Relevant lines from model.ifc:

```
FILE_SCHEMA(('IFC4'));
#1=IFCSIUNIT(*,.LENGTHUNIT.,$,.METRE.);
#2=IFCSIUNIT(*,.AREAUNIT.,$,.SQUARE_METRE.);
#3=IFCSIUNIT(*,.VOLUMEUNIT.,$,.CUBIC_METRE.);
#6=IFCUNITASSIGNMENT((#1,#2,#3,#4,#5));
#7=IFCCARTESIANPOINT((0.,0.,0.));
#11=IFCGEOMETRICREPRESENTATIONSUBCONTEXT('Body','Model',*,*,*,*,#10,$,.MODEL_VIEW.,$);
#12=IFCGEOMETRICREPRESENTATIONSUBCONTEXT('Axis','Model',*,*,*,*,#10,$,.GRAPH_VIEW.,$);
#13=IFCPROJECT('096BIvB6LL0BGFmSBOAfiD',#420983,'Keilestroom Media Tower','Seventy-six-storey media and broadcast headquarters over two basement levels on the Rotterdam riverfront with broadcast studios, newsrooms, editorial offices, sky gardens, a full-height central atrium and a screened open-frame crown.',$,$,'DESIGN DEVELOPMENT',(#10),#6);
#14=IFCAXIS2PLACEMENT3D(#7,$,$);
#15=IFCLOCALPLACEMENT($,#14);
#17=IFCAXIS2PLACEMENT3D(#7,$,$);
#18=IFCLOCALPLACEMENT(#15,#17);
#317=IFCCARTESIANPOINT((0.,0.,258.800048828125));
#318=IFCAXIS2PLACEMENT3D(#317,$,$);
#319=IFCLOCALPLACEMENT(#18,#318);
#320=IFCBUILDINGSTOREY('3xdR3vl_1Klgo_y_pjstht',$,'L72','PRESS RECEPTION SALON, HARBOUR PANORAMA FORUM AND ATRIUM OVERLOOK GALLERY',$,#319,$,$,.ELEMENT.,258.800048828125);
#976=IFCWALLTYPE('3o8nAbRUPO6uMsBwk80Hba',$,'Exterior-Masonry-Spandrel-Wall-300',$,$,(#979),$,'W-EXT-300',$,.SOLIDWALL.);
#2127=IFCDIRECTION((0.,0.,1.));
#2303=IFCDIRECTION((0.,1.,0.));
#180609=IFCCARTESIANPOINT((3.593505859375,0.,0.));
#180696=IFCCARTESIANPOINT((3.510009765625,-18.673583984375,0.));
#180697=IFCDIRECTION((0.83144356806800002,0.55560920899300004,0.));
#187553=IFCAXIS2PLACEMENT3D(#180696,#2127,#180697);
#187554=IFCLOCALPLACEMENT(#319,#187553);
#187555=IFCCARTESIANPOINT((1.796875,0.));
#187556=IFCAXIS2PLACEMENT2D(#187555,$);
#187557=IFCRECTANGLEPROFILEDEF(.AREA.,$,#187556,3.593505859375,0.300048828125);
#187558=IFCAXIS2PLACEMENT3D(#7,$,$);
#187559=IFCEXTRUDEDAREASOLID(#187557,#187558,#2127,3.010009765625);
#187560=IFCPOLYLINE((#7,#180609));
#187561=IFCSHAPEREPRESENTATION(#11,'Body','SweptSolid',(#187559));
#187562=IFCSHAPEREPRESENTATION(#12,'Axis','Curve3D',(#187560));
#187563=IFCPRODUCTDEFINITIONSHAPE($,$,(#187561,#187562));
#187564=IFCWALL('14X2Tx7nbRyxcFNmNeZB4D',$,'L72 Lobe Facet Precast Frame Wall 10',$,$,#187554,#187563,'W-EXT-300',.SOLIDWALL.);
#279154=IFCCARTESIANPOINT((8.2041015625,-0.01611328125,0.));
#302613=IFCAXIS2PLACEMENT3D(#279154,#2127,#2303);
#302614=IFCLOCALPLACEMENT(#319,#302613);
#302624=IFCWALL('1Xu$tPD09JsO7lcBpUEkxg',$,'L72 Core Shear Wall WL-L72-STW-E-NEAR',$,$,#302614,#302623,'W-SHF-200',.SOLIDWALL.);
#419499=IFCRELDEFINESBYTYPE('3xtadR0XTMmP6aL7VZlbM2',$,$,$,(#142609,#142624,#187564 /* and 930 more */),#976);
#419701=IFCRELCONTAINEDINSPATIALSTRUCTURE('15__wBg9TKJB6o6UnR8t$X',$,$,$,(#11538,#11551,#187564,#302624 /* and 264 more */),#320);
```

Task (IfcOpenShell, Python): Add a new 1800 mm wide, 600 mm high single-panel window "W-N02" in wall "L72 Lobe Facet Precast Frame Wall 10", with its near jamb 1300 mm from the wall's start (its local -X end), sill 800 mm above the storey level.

```python
import numpy as np
import ifcopenshell
import ifcopenshell.api.feature
import ifcopenshell.api.geometry
import ifcopenshell.api.root
import ifcopenshell.api.spatial
import ifcopenshell.geom
import ifcopenshell.util.element
import ifcopenshell.util.placement
import ifcopenshell.util.representation
import ifcopenshell.util.shape
import ifcopenshell.util.unit

model = ifcopenshell.open("model.ifc")
unit_scale = ifcopenshell.util.unit.calculate_unit_scale(model)
settings = ifcopenshell.geom.settings()


def volume(element):
    """Net volume in cubic metres, openings subtracted."""
    shape = ifcopenshell.geom.create_shape(settings, element)
    return ifcopenshell.util.shape.get_volume(shape.geometry)


wall = model.by_id(187564)
storey = ifcopenshell.util.element.get_container(wall, ifc_class="IfcBuildingStorey")
context = ifcopenshell.util.representation.get_context(model, "Model", "Body", "MODEL_VIEW")
before = volume(wall)

width, height, from_end, sill = 1.8, 0.6, 1.3, 0.8  # metres

# The wall runs along its own X axis, and the end named is its -X end.
wall_shape = ifcopenshell.geom.create_shape(settings, wall)
x, y, z = ifcopenshell.util.shape.get_vertices(wall_shape.geometry).T
start = x.min() + from_end
face, thickness = float(y.min()), float(y.max() - y.min())
wall_matrix = ifcopenshell.util.placement.get_local_placement(wall.ObjectPlacement)
level = ifcopenshell.util.placement.get_local_placement(storey.ObjectPlacement)[2, 3]


def in_wall(x, y):
    """Placement at x, y metres in the wall's axes, at sill height."""
    matrix = wall_matrix.copy()
    matrix[:, 3] = wall_matrix @ np.array([x / unit_scale, y / unit_scale, 0.0, 1.0])
    matrix[2, 3] = level + sill / unit_scale
    return matrix


# Opening: a box that overshoots both wall faces by 50 mm.
opening = ifcopenshell.api.root.create_entity(model, ifc_class="IfcOpeningElement", predefined_type="OPENING")
box = ifcopenshell.api.geometry.add_wall_representation(
    model, context=context, length=width, height=height, thickness=thickness + 0.1
)
ifcopenshell.api.geometry.assign_representation(model, product=opening, representation=box)
ifcopenshell.api.geometry.edit_object_placement(model, product=opening, matrix=in_wall(start, face - 0.05), is_si=False)
ifcopenshell.api.feature.add_feature(model, feature=opening, element=wall)

window = ifcopenshell.api.root.create_entity(model, ifc_class="IfcWindow", name="W-N02", predefined_type="WINDOW")
window.OverallWidth, window.OverallHeight = width / unit_scale, height / unit_scale
window.PartitioningType = "SINGLE_PANEL"
body = ifcopenshell.api.geometry.add_window_representation(
    model,
    context=context,
    overall_width=window.OverallWidth,
    overall_height=window.OverallHeight,
    partition_type="SINGLE_PANEL",
)
ifcopenshell.api.geometry.assign_representation(model, product=window, representation=body)
ifcopenshell.api.spatial.assign_container(model, products=[window], relating_structure=storey)
ifcopenshell.api.feature.add_filling(model, opening=opening, element=window)

# Centre the window in the wall's thickness.
ifcopenshell.api.geometry.edit_object_placement(model, product=window, matrix=in_wall(start, face), is_si=False)
window_shape = ifcopenshell.geom.create_shape(settings, window)
depth = ifcopenshell.util.shape.get_vertices(window_shape.geometry)[:, 1]
offset = face + thickness / 2 - (depth.min() + depth.max()) / 2
ifcopenshell.api.geometry.edit_object_placement(model, product=window, matrix=in_wall(start, offset), is_si=False)

after = volume(wall)

print(f"wall volume {before:.3f} -> {after:.3f} m3")

model.write("model_updated.ifc")
```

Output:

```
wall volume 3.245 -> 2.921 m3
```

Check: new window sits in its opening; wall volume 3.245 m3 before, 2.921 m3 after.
